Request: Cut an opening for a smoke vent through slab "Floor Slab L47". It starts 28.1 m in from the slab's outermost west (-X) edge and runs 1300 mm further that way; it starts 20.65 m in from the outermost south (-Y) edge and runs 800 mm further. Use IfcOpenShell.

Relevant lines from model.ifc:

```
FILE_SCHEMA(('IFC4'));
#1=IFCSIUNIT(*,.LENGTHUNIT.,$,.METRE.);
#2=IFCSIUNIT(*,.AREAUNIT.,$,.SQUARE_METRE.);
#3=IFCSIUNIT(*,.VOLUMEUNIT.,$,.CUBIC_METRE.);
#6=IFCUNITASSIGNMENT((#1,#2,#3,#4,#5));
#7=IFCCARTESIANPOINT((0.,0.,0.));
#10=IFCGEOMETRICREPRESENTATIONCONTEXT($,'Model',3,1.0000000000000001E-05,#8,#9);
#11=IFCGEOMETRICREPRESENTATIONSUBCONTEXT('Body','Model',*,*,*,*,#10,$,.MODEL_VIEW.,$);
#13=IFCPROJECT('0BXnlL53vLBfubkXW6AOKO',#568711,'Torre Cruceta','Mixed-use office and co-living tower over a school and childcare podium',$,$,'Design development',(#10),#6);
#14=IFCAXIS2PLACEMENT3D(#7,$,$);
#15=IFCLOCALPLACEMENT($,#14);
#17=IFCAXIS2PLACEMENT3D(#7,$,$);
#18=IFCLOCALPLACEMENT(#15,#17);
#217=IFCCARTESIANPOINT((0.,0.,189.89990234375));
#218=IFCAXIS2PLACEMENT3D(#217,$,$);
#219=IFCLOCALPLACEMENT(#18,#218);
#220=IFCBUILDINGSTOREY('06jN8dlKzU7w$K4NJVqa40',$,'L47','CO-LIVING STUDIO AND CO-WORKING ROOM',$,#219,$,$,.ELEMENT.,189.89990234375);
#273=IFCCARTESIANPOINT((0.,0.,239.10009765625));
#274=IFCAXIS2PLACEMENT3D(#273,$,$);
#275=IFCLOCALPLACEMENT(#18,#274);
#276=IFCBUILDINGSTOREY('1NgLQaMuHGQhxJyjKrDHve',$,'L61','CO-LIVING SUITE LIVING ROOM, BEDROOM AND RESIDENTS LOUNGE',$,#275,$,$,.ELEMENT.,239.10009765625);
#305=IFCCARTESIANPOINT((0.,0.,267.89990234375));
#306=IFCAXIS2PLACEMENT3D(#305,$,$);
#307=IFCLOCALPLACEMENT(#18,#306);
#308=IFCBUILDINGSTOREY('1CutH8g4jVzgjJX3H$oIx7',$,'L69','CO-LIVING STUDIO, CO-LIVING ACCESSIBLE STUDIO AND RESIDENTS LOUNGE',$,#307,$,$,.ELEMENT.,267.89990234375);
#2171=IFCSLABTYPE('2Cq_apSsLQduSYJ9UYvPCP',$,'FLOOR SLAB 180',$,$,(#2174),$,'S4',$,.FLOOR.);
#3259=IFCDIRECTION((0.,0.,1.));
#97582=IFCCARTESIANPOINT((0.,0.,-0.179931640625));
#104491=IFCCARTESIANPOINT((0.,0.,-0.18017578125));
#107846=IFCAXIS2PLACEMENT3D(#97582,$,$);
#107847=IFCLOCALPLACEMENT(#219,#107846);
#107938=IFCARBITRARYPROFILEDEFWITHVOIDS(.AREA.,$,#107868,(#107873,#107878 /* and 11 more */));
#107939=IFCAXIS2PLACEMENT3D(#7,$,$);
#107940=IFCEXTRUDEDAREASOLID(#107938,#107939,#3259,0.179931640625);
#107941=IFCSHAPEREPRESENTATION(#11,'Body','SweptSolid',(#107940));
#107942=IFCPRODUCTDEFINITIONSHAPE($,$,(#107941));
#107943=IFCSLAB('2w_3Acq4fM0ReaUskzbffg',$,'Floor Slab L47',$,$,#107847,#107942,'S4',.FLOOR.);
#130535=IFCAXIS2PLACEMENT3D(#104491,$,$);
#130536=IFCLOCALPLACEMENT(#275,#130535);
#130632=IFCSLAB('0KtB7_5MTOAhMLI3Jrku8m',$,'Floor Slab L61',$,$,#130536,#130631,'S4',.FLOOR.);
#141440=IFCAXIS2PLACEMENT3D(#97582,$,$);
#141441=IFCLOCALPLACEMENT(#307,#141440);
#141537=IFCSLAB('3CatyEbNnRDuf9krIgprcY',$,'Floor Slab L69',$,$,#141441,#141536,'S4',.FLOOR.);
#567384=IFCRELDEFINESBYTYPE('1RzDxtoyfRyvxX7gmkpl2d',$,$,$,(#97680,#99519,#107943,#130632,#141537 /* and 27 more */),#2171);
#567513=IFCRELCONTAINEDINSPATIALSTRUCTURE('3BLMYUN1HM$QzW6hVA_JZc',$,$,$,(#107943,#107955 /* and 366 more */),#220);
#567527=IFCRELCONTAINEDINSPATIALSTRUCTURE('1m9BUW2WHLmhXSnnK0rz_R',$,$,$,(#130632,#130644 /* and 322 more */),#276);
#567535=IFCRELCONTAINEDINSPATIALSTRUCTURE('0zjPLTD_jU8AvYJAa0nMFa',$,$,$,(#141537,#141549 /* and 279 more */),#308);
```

```python
import numpy as np
import ifcopenshell
import ifcopenshell.api.feature
import ifcopenshell.api.geometry
import ifcopenshell.api.root
import ifcopenshell.geom
import ifcopenshell.util.placement
import ifcopenshell.util.representation
import ifcopenshell.util.shape
import ifcopenshell.util.unit

model = ifcopenshell.open("model.ifc")
unit_scale = ifcopenshell.util.unit.calculate_unit_scale(model)
settings = ifcopenshell.geom.settings()


def volume(element):
    """Net volume in cubic metres, openings subtracted."""
    shape = ifcopenshell.geom.create_shape(settings, element)
    return ifcopenshell.util.shape.get_volume(shape.geometry)


slab = model.by_id(107943)
before = volume(slab)

# Extent in the slab's own axes, in metres. The edges named are its -X and -Y sides.
slab_shape = ifcopenshell.geom.create_shape(settings, slab)
vertices = ifcopenshell.util.shape.get_vertices(slab_shape.geometry)
x_min, y_min, bottom = vertices.min(axis=0)
top = vertices[:, 2].max()

opening = ifcopenshell.api.root.create_entity(model, ifc_class="IfcOpeningElement", name="Smoke vent opening", predefined_type="OPENING")
context = ifcopenshell.util.representation.get_context(model, "Model", "Body", "MODEL_VIEW")
width, depth = 1.3, 0.8
outline = [(0.0, 0.0), (width, 0.0), (width, depth), (0.0, depth), (0.0, 0.0)]
# Overshoot both faces by 50 mm so the cut is clean.
shape = ifcopenshell.api.geometry.add_slab_representation(
    model, context=context, depth=top - bottom + 0.1, polyline=outline
)
ifcopenshell.api.geometry.assign_representation(model, product=opening, representation=shape)

matrix = ifcopenshell.util.placement.get_local_placement(slab.ObjectPlacement)
matrix[:, 3] = matrix @ np.append(np.array([x_min + 28.1, y_min + 20.65, bottom - 0.05]) / unit_scale, 1.0)
ifcopenshell.api.geometry.edit_object_placement(model, product=opening, matrix=matrix, is_si=False)
ifcopenshell.api.feature.add_feature(model, feature=opening, element=slab)

after = volume(slab)

print(f"slab volume {before:.3f} -> {after:.3f} m3")

model.write("model_v2.ifc")
```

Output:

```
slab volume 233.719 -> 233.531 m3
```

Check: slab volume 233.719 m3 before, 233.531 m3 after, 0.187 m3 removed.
